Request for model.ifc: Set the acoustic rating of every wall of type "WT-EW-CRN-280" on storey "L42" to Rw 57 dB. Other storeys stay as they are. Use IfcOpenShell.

First a look at what the model holds.

```python
import ifcopenshell
import ifcopenshell.util.element

model = ifcopenshell.open("model.ifc")
print(model.schema)
storey = next(s for s in model.by_type("IfcBuildingStorey") if s.Name == "L42")
walls = [e for e in ifcopenshell.util.element.get_decomposition(storey) if e.is_a("IfcWall")]
seen = {}
for e in walls:
    element_type = ifcopenshell.util.element.get_type(e)
    key = (element_type.Name if element_type != e and element_type else None, ifcopenshell.util.element.get_pset(e, "Pset_WallCommon", "AcousticRating"))
    seen[key] = seen.get(key, 0) + 1
for (name, value), count in sorted(seen.items(), key=str):
    print(count, "x", name, "|", value)
```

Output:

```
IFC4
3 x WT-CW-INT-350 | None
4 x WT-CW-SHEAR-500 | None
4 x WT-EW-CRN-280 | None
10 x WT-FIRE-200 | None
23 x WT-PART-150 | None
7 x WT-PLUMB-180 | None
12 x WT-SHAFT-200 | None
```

```python
import ifcopenshell
import ifcopenshell.api.pset
import ifcopenshell.util.element

model = ifcopenshell.open("model.ifc")

storey = next(s for s in model.by_type("IfcBuildingStorey") if s.Name == "L42")
walls = [e for e in ifcopenshell.util.element.get_decomposition(storey) if e.is_a("IfcWall")]

count = 0
for e in walls:
    element_type = ifcopenshell.util.element.get_type(e)
    if element_type in (None, e) or element_type.Name != "WT-EW-CRN-280":
        continue
    found = ifcopenshell.util.element.get_pset(e, "Pset_WallCommon", should_inherit=False)
    if found:
        pset = model.by_id(found["id"])
        if len(ifcopenshell.util.element.get_elements_by_pset(pset)) > 1:
            pset = ifcopenshell.api.pset.unshare_pset(model, products=[e], pset=pset)[0]
    else:
        pset = ifcopenshell.api.pset.add_pset(model, product=e, name="Pset_WallCommon")
    ifcopenshell.api.pset.edit_pset(model, pset=pset, properties={"AcousticRating": "Rw 57 dB"})
    count += 1

print(count, "walls updated")

model.write("model_v2.ifc")
```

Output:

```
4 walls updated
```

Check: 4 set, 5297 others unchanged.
